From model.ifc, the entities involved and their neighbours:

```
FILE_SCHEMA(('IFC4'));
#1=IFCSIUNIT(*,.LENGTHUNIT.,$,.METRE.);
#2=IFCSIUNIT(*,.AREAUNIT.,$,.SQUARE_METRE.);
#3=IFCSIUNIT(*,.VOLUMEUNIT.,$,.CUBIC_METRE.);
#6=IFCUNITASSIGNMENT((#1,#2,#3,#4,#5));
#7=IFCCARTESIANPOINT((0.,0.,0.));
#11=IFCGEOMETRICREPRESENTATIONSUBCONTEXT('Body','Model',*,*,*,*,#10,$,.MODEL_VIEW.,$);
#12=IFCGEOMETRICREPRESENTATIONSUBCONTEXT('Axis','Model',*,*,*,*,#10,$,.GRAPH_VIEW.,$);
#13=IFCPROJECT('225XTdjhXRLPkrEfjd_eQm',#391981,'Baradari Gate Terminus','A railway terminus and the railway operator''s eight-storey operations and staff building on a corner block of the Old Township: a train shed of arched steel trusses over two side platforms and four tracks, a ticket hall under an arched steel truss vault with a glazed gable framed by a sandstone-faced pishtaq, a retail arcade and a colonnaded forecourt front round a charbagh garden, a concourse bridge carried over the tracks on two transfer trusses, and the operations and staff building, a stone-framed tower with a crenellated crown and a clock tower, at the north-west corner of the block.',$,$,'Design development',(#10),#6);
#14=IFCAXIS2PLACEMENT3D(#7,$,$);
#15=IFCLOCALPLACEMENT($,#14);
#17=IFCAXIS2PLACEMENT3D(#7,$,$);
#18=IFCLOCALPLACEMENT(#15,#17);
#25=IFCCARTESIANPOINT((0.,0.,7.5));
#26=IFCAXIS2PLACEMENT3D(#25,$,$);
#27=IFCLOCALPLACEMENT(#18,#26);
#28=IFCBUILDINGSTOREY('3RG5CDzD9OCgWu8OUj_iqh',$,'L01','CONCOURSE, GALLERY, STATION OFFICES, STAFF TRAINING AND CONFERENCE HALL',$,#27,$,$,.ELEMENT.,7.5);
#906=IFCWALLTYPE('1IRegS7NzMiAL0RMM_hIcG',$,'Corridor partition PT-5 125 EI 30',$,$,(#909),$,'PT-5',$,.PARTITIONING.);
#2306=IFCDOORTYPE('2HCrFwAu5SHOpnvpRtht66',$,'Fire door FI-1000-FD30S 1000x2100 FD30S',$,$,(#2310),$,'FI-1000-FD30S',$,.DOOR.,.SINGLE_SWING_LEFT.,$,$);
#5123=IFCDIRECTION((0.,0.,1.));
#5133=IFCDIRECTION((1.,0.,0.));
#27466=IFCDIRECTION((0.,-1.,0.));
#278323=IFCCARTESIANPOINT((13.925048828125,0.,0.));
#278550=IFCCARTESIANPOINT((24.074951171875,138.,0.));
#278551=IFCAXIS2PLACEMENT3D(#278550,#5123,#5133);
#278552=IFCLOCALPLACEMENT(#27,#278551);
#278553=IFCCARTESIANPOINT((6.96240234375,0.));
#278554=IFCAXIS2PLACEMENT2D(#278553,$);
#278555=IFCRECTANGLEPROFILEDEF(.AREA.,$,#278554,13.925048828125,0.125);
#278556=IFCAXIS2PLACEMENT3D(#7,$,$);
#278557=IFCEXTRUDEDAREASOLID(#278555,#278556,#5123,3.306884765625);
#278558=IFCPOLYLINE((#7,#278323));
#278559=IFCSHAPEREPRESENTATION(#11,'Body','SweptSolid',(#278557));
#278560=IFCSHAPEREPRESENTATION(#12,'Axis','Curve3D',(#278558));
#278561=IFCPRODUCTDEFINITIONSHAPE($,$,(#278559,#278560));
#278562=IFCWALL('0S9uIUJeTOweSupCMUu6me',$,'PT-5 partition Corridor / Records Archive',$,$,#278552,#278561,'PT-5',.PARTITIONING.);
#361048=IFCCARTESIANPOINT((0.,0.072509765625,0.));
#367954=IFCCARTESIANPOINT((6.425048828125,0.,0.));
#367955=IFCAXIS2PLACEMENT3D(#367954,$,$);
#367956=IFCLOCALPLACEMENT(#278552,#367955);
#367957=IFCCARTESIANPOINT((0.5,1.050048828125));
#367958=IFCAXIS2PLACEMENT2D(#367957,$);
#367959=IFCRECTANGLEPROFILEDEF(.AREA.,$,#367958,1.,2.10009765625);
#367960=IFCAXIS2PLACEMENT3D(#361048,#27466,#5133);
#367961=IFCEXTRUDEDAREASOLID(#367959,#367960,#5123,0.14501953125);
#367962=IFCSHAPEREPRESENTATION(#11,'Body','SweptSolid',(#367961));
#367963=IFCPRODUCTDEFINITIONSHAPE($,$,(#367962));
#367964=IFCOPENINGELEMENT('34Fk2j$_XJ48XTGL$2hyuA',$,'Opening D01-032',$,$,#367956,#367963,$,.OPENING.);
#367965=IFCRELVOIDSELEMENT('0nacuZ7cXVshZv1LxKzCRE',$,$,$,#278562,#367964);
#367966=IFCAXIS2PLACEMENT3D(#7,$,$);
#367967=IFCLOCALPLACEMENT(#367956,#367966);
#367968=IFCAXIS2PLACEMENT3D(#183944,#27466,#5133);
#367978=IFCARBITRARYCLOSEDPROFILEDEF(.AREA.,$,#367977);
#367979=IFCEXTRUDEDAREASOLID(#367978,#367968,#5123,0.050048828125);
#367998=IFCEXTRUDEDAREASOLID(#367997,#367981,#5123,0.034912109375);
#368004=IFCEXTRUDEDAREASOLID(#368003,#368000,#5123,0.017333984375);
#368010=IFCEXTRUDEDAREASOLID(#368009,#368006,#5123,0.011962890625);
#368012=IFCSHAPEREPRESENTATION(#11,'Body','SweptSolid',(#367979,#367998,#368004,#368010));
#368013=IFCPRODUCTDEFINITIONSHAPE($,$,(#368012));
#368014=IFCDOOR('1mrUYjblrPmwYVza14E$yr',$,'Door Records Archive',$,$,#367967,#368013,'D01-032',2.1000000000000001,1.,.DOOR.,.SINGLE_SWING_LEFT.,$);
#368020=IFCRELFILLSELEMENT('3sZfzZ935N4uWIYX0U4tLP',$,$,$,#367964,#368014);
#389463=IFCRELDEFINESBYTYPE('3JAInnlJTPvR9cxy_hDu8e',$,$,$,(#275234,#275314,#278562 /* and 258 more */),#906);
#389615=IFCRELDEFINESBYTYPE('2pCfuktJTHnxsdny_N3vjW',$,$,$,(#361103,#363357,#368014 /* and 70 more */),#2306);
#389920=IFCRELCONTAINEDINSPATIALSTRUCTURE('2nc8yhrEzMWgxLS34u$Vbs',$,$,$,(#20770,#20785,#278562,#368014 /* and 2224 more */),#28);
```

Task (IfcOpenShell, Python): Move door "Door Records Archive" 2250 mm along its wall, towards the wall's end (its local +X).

```python
import ifcopenshell
import ifcopenshell.api.geometry
import ifcopenshell.util.placement
import ifcopenshell.util.unit

model = ifcopenshell.open("model.ifc")
unit_scale = ifcopenshell.util.unit.calculate_unit_scale(model)

door = model.by_id(368014)
opening = door.FillsVoids[0].RelatingOpeningElement
wall = opening.VoidsElements[0].RelatingBuildingElement

wall_matrix = ifcopenshell.util.placement.get_local_placement(wall.ObjectPlacement)
shift = wall_matrix[:3, 0] * 2.25 / unit_scale
before = ifcopenshell.util.placement.get_local_placement(door.ObjectPlacement)[:3, 3].copy()

# The door is placed relative to its opening, so it follows when the opening moves.
matrix = ifcopenshell.util.placement.get_local_placement(opening.ObjectPlacement)
matrix[:3, 3] += shift
ifcopenshell.api.geometry.edit_object_placement(
    model, product=opening, matrix=matrix, is_si=False, should_transform_children=True
)

after = ifcopenshell.util.placement.get_local_placement(door.ObjectPlacement)[:3, 3]
print("door moved by", (after - before).round(3) + 0.0)

model.write("model_updated.ifc")
```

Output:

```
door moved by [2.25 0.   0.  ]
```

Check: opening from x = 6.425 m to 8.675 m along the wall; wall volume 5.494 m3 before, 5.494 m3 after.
